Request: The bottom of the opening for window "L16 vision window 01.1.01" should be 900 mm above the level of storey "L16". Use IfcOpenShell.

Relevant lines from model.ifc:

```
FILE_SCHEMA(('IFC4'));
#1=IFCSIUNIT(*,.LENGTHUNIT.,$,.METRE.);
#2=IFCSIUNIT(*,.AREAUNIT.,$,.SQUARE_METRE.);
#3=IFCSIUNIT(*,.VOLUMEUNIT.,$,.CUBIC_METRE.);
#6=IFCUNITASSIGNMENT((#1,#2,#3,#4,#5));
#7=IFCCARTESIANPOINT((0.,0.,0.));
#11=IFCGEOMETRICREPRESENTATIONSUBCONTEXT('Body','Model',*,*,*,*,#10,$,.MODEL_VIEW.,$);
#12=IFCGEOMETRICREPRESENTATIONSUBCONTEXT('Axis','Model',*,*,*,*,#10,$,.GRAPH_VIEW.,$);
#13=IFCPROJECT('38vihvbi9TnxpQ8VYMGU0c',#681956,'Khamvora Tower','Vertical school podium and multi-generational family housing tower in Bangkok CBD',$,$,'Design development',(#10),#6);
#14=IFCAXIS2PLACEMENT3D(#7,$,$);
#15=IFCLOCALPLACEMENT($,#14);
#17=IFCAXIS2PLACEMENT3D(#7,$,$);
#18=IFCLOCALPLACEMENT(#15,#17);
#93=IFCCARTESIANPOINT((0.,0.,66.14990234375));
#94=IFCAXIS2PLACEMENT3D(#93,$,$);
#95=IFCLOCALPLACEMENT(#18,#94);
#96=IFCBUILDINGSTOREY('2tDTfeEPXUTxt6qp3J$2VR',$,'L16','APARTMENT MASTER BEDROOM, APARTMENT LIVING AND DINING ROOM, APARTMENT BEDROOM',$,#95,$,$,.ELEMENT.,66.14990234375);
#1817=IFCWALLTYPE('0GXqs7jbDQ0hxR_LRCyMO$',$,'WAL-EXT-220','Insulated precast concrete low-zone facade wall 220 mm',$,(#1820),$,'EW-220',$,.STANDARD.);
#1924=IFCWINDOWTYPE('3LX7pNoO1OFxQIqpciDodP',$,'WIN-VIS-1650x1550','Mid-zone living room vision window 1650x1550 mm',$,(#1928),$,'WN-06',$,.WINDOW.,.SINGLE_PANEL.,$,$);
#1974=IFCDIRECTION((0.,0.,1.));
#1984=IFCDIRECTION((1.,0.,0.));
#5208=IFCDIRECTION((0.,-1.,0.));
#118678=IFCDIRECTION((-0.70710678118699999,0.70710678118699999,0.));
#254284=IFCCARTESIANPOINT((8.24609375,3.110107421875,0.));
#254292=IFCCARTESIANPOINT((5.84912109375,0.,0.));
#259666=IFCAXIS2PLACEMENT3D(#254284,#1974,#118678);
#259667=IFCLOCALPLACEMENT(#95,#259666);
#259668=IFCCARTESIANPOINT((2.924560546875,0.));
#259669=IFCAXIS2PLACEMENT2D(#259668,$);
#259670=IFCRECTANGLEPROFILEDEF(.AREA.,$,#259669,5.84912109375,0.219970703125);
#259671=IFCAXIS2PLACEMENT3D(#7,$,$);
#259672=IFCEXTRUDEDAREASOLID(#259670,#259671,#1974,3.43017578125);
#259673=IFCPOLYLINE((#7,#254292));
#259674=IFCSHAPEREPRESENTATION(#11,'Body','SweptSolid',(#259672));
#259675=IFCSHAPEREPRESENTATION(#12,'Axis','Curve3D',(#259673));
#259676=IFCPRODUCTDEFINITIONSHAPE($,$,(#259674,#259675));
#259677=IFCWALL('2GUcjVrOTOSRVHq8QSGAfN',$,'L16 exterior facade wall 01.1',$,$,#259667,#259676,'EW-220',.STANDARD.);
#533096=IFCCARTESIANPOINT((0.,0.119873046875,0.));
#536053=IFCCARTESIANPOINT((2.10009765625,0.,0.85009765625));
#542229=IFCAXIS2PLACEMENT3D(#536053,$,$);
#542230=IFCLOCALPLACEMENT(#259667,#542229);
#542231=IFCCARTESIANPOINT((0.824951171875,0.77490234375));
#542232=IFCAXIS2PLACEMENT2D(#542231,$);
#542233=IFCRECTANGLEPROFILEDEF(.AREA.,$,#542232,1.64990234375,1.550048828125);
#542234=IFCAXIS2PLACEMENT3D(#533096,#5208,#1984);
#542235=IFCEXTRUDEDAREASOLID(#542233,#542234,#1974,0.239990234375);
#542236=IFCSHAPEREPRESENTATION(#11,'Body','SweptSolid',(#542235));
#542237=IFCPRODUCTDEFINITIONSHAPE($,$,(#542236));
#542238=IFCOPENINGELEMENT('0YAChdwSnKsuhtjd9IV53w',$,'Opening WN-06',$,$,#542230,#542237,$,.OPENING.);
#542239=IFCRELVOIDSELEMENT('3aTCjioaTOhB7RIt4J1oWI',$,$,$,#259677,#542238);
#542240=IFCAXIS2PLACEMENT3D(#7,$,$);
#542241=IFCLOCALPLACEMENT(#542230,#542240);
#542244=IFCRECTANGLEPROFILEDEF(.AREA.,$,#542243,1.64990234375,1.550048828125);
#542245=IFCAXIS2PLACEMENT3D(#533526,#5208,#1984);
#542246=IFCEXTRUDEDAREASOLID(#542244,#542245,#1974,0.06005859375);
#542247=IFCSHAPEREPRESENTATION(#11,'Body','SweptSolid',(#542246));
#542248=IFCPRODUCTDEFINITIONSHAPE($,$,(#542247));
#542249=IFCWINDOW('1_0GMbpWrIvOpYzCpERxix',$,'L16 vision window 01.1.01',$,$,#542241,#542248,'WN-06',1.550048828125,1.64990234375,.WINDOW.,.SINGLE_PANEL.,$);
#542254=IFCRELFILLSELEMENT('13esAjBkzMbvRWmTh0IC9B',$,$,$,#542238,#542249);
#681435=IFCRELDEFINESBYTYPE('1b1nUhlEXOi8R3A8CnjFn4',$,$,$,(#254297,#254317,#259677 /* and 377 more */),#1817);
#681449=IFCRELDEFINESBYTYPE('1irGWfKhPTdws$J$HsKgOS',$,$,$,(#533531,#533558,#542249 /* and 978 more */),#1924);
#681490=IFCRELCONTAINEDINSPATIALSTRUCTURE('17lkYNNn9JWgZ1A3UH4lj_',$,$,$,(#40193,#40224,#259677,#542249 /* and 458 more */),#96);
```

```python
import numpy as np
import ifcopenshell
import ifcopenshell.api.geometry
import ifcopenshell.geom
import ifcopenshell.util.element
import ifcopenshell.util.placement
import ifcopenshell.util.shape
import ifcopenshell.util.unit

model = ifcopenshell.open("model.ifc")
unit_scale = ifcopenshell.util.unit.calculate_unit_scale(model)

window = model.by_guid("1_0GMbpWrIvOpYzCpERxix")
opening = window.FillsVoids[0].RelatingOpeningElement
storey = ifcopenshell.util.element.get_container(window, ifc_class="IfcBuildingStorey")
level = ifcopenshell.util.placement.get_local_placement(storey.ObjectPlacement)[2, 3]

# The opening's origin need not be at the sill, so measure its lowest point.
shape = ifcopenshell.geom.create_shape(ifcopenshell.geom.settings(), opening)
bottom = ifcopenshell.util.shape.get_shape_bottom_elevation(shape, shape.geometry) / unit_scale
dz = level + 0.9 / unit_scale - bottom

shift = np.array([0.0, 0.0, dz])
# The window is placed relative to its opening, so it follows when the opening moves.
matrix = ifcopenshell.util.placement.get_local_placement(opening.ObjectPlacement)
matrix[:3, 3] += shift
ifcopenshell.api.geometry.edit_object_placement(
    model, product=opening, matrix=matrix, is_si=False, should_transform_children=True
)

print(f"moved by {dz * unit_scale:+.3f} m")

model.write("model_edited.ifc")
```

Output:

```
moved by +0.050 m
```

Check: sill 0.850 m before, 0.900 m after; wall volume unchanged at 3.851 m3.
